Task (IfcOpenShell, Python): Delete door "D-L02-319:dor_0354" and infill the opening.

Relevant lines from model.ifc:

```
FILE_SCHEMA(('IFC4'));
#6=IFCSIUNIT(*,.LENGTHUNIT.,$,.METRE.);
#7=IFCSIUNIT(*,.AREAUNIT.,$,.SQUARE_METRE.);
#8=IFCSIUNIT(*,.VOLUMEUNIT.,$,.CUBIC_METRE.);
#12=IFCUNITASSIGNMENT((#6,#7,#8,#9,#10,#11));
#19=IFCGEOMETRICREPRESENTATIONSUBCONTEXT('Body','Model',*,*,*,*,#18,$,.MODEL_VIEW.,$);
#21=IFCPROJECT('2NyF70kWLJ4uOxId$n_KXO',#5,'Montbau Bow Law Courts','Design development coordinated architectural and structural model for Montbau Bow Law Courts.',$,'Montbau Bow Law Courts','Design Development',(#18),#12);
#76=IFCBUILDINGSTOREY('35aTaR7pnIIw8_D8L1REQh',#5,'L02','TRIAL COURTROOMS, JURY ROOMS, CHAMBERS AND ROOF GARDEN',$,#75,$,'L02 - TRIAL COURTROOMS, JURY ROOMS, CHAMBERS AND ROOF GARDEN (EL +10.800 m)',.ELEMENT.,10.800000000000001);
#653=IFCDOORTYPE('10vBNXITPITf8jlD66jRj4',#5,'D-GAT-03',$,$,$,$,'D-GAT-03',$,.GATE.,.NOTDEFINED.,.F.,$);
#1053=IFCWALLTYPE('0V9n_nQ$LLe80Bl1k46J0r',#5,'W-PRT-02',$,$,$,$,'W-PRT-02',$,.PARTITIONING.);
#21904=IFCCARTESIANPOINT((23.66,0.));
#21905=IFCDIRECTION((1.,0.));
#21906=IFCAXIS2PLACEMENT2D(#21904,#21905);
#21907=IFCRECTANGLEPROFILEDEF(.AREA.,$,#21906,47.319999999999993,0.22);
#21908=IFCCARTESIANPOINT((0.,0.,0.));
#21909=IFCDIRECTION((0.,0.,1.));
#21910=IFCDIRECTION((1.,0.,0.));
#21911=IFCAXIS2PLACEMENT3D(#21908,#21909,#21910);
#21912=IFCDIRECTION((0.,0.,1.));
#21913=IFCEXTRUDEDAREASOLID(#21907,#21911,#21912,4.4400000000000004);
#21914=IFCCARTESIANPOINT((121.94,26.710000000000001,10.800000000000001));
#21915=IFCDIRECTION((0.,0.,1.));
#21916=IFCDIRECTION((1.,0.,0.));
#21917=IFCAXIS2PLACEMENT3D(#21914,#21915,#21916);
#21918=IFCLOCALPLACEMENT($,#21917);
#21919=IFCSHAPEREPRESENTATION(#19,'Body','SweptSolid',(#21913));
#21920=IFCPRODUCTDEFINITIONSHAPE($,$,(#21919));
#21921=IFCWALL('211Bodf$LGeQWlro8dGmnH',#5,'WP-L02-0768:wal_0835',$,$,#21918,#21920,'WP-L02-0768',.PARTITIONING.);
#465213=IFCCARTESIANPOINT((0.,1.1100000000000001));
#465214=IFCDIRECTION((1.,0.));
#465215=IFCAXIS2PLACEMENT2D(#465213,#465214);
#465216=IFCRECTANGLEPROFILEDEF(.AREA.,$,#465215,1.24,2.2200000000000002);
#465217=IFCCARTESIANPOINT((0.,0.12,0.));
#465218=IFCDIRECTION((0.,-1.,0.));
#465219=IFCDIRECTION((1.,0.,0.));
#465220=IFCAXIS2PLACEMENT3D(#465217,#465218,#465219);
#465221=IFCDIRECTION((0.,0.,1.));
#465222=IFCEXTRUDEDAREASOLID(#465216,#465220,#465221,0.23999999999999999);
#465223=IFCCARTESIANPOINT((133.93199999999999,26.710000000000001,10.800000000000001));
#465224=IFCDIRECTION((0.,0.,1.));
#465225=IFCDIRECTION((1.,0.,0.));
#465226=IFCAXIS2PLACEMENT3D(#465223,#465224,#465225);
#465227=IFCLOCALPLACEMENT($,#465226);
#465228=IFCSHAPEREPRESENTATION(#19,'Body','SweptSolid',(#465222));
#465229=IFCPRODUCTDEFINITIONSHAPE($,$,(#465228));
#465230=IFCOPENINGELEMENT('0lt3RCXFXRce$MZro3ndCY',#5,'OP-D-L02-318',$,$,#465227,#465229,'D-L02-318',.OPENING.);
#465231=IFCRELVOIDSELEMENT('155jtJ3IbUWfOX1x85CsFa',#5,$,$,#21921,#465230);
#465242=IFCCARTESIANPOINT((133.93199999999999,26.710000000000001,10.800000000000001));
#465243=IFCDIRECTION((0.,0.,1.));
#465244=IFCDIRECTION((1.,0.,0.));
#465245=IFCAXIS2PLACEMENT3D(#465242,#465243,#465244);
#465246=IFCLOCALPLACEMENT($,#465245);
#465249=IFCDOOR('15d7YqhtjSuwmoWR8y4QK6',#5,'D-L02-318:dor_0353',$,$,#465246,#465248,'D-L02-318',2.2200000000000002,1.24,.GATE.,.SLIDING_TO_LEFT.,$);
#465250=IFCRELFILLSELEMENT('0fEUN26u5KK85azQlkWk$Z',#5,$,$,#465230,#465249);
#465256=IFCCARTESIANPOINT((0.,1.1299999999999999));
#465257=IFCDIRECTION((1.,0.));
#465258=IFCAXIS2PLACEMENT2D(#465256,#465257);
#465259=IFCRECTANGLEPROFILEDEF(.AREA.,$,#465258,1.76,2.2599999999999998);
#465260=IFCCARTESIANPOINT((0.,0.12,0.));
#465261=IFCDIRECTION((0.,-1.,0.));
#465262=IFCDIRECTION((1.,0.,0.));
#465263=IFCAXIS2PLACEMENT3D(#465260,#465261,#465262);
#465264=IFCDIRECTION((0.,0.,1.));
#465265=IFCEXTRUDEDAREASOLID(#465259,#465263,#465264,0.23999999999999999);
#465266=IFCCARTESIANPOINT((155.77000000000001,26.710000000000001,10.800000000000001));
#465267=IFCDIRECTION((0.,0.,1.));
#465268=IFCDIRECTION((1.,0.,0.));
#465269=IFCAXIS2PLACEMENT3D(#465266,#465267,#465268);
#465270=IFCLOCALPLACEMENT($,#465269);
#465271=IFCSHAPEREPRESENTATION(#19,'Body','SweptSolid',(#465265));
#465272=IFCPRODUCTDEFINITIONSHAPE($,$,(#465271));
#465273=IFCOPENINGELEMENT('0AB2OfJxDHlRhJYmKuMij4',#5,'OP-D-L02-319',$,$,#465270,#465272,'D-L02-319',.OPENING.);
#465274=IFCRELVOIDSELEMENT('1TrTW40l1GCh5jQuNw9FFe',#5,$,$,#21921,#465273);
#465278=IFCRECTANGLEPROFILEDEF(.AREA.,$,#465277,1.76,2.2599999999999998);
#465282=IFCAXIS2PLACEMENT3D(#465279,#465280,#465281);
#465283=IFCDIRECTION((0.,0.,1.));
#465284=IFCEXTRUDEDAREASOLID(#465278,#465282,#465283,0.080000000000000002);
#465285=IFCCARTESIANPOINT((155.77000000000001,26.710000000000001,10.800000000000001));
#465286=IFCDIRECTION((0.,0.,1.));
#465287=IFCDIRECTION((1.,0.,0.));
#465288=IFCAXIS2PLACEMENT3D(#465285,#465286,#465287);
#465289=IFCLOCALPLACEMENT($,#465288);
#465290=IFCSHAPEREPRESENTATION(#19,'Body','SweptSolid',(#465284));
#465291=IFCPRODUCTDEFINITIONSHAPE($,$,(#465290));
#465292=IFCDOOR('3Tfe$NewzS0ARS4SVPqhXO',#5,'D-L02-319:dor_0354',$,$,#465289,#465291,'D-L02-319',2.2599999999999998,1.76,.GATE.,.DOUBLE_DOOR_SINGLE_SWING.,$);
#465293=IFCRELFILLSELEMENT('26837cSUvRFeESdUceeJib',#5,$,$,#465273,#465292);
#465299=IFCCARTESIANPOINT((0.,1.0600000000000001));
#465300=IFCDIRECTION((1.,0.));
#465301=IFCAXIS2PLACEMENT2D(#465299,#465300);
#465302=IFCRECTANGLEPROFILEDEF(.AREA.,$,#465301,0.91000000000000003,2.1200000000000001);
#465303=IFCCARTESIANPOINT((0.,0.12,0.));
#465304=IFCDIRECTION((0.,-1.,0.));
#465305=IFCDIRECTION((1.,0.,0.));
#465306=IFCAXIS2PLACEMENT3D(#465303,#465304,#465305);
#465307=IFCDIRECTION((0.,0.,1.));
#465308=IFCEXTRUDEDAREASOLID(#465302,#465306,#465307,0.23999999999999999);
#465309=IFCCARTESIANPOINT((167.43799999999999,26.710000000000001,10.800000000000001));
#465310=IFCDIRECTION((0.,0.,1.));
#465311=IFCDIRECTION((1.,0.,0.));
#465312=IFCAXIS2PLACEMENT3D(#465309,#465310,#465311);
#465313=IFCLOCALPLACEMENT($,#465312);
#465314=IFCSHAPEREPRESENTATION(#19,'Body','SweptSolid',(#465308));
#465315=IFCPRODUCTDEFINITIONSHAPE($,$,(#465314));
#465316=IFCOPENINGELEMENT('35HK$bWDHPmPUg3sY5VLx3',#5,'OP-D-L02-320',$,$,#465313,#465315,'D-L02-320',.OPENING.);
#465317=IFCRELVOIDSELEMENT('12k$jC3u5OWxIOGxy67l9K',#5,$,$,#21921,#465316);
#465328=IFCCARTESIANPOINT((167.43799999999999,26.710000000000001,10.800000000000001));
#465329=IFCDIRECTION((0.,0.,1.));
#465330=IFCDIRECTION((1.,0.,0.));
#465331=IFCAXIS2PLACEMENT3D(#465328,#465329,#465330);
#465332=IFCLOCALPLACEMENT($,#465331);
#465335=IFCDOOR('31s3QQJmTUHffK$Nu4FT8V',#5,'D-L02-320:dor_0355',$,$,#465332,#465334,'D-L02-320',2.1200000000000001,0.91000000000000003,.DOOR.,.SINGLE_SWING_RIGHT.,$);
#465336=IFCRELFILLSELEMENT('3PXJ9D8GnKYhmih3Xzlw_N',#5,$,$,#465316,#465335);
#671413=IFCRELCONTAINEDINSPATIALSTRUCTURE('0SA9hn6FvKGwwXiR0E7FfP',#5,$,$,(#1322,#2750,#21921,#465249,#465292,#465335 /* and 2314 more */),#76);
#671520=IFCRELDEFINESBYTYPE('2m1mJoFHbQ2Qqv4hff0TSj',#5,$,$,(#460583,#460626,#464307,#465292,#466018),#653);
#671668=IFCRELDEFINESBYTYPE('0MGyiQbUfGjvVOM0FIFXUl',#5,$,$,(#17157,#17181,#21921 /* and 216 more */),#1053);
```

```python
import ifcopenshell
import ifcopenshell.api.feature
import ifcopenshell.api.root
import ifcopenshell.geom
import ifcopenshell.util.shape

model = ifcopenshell.open("model.ifc")
settings = ifcopenshell.geom.settings()


def volume(element):
    """Net volume in cubic metres, openings subtracted."""
    shape = ifcopenshell.geom.create_shape(settings, element)
    return ifcopenshell.util.shape.get_volume(shape.geometry)


door = model.by_guid("3Tfe$NewzS0ARS4SVPqhXO")
opening = door.FillsVoids[0].RelatingOpeningElement
wall = opening.VoidsElements[0].RelatingBuildingElement
before = volume(wall)

ifcopenshell.api.root.remove_product(model, product=door)
ifcopenshell.api.feature.remove_feature(model, feature=opening)

after = volume(wall)

print(f"wall volume {before:.3f} -> {after:.3f} m3")

model.write("model_updated.ifc")
```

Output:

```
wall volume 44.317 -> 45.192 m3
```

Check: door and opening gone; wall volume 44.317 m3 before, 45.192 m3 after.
